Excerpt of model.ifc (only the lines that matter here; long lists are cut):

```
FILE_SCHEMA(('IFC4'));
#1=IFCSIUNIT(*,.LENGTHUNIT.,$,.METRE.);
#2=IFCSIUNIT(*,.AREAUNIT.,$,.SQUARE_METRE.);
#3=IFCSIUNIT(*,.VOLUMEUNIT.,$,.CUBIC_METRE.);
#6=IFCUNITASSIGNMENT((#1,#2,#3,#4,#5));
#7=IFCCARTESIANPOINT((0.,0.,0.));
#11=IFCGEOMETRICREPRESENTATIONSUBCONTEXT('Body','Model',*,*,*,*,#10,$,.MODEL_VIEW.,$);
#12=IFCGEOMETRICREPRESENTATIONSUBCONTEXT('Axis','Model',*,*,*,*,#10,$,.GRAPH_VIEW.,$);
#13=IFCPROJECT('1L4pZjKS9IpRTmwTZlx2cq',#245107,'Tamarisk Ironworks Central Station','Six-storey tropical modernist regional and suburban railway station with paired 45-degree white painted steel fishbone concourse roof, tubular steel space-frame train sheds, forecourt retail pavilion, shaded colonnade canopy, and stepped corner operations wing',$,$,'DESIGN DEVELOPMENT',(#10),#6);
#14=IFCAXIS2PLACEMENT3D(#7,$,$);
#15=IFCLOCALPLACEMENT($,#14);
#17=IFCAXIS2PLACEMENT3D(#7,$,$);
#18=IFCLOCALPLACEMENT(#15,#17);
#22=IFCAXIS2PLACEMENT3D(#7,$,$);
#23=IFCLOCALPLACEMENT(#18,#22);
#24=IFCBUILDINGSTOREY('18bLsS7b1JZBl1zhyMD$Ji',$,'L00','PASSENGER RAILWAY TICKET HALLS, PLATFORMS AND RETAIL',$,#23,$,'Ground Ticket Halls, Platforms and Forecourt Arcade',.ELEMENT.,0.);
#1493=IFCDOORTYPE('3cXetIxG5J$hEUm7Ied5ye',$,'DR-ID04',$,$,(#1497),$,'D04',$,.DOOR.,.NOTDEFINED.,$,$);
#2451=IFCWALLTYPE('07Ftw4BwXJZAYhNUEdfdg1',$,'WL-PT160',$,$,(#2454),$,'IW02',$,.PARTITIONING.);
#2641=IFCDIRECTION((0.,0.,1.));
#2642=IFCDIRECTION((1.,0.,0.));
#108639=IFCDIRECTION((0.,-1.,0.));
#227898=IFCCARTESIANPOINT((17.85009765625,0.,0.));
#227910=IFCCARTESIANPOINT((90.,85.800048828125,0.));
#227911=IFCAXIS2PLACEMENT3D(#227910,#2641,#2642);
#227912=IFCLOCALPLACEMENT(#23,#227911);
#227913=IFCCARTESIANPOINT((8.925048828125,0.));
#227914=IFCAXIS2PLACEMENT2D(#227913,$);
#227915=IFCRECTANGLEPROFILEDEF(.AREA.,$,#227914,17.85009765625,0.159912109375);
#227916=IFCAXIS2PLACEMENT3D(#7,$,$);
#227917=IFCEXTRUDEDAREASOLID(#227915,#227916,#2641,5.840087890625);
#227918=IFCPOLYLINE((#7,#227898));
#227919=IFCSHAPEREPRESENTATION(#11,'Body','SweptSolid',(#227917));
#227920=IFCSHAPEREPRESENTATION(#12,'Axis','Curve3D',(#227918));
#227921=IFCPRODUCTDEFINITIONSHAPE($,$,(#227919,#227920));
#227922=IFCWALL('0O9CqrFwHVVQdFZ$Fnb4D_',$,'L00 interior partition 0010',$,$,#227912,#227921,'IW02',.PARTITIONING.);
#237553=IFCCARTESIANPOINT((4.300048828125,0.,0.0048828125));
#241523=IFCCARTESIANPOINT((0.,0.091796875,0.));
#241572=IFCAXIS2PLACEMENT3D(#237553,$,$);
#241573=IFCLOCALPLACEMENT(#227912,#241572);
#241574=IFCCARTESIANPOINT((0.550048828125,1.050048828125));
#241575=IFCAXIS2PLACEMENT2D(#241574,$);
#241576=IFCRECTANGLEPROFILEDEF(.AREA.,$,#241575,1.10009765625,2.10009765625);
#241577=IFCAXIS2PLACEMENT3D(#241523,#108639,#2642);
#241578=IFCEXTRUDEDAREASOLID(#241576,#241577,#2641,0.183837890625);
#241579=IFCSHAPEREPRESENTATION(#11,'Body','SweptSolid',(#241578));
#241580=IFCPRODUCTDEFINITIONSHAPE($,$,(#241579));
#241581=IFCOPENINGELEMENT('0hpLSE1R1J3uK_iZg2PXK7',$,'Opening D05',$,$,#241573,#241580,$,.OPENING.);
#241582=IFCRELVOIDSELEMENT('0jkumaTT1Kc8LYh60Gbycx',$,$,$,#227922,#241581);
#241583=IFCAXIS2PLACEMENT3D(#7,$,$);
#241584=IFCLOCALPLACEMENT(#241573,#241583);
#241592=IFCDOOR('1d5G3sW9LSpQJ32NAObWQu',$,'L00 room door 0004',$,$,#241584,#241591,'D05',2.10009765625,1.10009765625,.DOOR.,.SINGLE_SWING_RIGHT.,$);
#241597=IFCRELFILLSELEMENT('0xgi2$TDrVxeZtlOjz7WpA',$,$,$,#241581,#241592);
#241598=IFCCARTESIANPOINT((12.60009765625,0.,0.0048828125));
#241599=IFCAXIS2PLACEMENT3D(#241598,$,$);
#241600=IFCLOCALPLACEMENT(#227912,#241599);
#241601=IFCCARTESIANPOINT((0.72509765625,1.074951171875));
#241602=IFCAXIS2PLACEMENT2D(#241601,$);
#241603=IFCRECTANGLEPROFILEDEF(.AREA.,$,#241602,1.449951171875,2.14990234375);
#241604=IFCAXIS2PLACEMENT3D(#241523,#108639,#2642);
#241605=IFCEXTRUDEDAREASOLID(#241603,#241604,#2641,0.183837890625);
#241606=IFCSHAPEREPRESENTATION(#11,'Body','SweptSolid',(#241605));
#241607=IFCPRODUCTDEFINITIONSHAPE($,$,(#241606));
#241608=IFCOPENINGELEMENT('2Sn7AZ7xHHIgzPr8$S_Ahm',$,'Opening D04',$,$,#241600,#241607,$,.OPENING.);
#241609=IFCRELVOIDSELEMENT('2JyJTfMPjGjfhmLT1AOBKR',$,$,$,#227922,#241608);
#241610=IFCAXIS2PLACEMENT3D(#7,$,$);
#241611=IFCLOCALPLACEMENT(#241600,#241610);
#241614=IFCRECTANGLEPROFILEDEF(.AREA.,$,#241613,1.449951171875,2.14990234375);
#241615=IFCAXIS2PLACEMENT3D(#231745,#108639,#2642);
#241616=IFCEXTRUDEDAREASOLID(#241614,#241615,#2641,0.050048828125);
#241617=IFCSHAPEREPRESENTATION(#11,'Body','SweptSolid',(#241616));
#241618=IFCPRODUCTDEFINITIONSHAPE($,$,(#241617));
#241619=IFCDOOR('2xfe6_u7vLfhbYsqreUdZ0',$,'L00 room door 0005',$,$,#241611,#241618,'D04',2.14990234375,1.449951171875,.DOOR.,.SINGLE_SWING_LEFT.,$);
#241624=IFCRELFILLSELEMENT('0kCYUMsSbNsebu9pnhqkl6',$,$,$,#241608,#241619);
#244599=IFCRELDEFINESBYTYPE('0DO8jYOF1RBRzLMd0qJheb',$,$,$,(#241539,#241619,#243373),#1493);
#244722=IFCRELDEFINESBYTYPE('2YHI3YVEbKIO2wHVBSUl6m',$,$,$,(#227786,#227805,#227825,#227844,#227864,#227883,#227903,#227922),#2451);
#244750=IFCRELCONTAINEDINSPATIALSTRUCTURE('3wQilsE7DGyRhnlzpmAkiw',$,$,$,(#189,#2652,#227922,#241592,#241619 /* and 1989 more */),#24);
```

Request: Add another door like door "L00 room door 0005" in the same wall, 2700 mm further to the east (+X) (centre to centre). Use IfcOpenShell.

```python
import ifcopenshell
import ifcopenshell.api.feature
import ifcopenshell.api.geometry
import ifcopenshell.api.root
import ifcopenshell.geom
import ifcopenshell.util.element
import ifcopenshell.util.placement
import ifcopenshell.util.shape
import ifcopenshell.util.unit

model = ifcopenshell.open("model.ifc")
unit_scale = ifcopenshell.util.unit.calculate_unit_scale(model)
settings = ifcopenshell.geom.settings()


def volume(element):
    """Net volume in cubic metres, openings subtracted."""
    shape = ifcopenshell.geom.create_shape(settings, element)
    return ifcopenshell.util.shape.get_volume(shape.geometry)


door = model.by_id(241619)
opening = door.FillsVoids[0].RelatingOpeningElement
wall = opening.VoidsElements[0].RelatingBuildingElement
before = volume(wall)
shift = ifcopenshell.util.placement.get_local_placement(wall.ObjectPlacement)[:3, 0] * 2.7 / unit_scale

# copy_class copies the void relationship, type, container and properties, but no geometry.
new_opening = ifcopenshell.api.root.copy_class(model, product=opening)
new_opening.Representation = ifcopenshell.util.element.copy_deep(
    model, opening.Representation, exclude=["IfcGeometricRepresentationContext", "IfcRepresentationMap"]
)
new_door = ifcopenshell.api.root.copy_class(model, product=door)
new_door.Representation = ifcopenshell.util.element.copy_deep(
    model, door.Representation, exclude=["IfcGeometricRepresentationContext", "IfcRepresentationMap"]
)
new_door.Tag = None
ifcopenshell.api.feature.add_filling(model, opening=new_opening, element=new_door)

for old, new in ((opening, new_opening), (door, new_door)):
    matrix = ifcopenshell.util.placement.get_local_placement(old.ObjectPlacement)
    matrix[:3, 3] += shift
    ifcopenshell.api.geometry.edit_object_placement(model, product=new, matrix=matrix, is_si=False)

after = volume(wall)

print(f"wall volume {before:.3f} -> {after:.3f} m3")

model.write("model_rev.ifc")
```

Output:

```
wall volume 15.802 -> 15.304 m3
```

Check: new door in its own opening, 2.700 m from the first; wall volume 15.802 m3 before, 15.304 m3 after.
